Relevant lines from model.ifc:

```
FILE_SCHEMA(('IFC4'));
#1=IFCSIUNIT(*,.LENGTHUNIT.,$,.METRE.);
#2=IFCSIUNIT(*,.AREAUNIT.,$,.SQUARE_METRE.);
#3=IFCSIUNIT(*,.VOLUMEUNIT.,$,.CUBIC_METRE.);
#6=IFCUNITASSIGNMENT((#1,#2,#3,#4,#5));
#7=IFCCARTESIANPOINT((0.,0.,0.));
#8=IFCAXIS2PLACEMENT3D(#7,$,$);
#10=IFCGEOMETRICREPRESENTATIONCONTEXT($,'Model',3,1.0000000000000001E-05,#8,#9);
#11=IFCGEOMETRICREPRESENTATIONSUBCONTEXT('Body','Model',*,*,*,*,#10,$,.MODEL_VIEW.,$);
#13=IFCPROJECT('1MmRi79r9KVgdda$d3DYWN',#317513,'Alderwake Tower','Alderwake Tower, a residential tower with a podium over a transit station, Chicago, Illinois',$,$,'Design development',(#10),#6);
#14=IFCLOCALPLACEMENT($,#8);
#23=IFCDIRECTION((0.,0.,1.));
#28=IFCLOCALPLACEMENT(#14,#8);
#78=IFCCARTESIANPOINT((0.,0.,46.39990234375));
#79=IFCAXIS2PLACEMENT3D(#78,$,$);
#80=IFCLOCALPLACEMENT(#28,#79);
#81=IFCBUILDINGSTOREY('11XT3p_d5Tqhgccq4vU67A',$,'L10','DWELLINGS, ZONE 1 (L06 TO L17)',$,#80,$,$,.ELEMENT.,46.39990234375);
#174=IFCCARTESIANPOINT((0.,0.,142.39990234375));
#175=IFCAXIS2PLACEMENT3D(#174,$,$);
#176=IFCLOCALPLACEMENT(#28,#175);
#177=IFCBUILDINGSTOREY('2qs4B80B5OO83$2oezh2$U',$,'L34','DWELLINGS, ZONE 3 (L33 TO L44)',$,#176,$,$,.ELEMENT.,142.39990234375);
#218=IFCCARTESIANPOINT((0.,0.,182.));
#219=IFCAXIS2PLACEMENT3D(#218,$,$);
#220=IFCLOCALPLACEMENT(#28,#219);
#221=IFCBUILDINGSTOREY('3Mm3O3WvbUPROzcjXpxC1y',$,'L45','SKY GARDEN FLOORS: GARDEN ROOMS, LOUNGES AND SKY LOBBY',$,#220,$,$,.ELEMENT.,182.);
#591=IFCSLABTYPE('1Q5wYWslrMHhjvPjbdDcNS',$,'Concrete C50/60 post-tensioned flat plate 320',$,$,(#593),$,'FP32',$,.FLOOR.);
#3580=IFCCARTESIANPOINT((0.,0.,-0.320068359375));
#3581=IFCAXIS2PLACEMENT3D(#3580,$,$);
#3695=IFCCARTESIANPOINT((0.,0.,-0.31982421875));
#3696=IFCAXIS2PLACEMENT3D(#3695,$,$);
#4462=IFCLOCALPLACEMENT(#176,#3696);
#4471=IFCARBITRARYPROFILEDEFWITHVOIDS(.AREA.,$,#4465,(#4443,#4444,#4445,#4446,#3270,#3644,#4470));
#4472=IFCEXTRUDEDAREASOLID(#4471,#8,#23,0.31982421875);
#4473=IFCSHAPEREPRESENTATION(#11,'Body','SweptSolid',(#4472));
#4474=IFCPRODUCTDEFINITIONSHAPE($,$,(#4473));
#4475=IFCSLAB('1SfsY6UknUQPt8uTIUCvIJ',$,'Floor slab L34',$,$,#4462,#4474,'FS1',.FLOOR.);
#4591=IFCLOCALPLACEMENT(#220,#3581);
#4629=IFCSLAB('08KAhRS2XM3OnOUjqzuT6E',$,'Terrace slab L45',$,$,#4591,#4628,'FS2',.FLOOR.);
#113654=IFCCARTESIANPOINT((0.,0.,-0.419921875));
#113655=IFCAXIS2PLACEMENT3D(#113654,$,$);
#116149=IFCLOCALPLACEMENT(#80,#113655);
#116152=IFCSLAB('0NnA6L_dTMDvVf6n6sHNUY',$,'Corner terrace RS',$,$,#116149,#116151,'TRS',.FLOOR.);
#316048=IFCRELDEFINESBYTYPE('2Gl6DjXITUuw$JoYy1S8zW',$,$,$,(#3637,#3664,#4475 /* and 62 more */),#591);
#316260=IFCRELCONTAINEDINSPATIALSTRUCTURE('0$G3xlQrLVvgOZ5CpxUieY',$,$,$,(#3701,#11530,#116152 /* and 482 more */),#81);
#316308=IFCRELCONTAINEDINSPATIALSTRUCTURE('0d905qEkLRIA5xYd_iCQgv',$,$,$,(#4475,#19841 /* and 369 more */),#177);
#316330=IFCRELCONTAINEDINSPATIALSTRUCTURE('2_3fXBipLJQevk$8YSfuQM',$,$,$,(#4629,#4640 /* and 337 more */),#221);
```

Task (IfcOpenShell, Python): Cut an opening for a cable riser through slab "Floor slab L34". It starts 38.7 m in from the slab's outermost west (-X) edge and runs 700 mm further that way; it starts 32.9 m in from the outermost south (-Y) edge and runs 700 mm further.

```python
import numpy as np
import ifcopenshell
import ifcopenshell.api.feature
import ifcopenshell.api.geometry
import ifcopenshell.api.root
import ifcopenshell.geom
import ifcopenshell.util.placement
import ifcopenshell.util.representation
import ifcopenshell.util.shape
import ifcopenshell.util.unit

model = ifcopenshell.open("model.ifc")
unit_scale = ifcopenshell.util.unit.calculate_unit_scale(model)
settings = ifcopenshell.geom.settings()


def volume(element):
    """Net volume in cubic metres, openings subtracted."""
    shape = ifcopenshell.geom.create_shape(settings, element)
    return ifcopenshell.util.shape.get_volume(shape.geometry)


slab = model.by_id(4475)
before = volume(slab)

# Extent in the slab's own axes, in metres. The edges named are its -X and -Y sides.
slab_shape = ifcopenshell.geom.create_shape(settings, slab)
vertices = ifcopenshell.util.shape.get_vertices(slab_shape.geometry)
x_min, y_min, bottom = vertices.min(axis=0)
top = vertices[:, 2].max()

opening = ifcopenshell.api.root.create_entity(model, ifc_class="IfcOpeningElement", name="Cable riser opening", predefined_type="OPENING")
context = ifcopenshell.util.representation.get_context(model, "Model", "Body", "MODEL_VIEW")
width, depth = 0.7, 0.7
outline = [(0.0, 0.0), (width, 0.0), (width, depth), (0.0, depth), (0.0, 0.0)]
# Overshoot both faces by 50 mm so the cut is clean.
shape = ifcopenshell.api.geometry.add_slab_representation(
    model, context=context, depth=top - bottom + 0.1, polyline=outline
)
ifcopenshell.api.geometry.assign_representation(model, product=opening, representation=shape)

matrix = ifcopenshell.util.placement.get_local_placement(slab.ObjectPlacement)
matrix[:, 3] = matrix @ np.append(np.array([x_min + 38.7, y_min + 32.9, bottom - 0.05]) / unit_scale, 1.0)
ifcopenshell.api.geometry.edit_object_placement(model, product=opening, matrix=matrix, is_si=False)
ifcopenshell.api.feature.add_feature(model, feature=opening, element=slab)

after = volume(slab)

print(f"slab volume {before:.3f} -> {after:.3f} m3")

model.write("model_edited.ifc")
```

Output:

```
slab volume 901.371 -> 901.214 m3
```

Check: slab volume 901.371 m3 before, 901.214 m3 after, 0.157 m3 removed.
